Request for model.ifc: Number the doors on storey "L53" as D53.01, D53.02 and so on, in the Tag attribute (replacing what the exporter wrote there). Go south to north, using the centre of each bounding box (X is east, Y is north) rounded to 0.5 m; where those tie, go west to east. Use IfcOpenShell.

First a look at what the model holds.

```python
import ifcopenshell
import ifcopenshell.util.element
import ifcopenshell.util.placement

model = ifcopenshell.open("model.ifc")
print(model.schema)
storey = next(s for s in model.by_type("IfcBuildingStorey") if s.Name == "L53")
doors = [e for e in ifcopenshell.util.element.get_decomposition(storey) if e.is_a("IfcDoor")]
for e in sorted(doors, key=lambda e: e.id()):
    origin = ifcopenshell.util.placement.get_local_placement(e.ObjectPlacement)[:3, 3]
    print(e.id(), e.Tag, e.Name, origin.round(2) + 0.0, sep=" | ")
```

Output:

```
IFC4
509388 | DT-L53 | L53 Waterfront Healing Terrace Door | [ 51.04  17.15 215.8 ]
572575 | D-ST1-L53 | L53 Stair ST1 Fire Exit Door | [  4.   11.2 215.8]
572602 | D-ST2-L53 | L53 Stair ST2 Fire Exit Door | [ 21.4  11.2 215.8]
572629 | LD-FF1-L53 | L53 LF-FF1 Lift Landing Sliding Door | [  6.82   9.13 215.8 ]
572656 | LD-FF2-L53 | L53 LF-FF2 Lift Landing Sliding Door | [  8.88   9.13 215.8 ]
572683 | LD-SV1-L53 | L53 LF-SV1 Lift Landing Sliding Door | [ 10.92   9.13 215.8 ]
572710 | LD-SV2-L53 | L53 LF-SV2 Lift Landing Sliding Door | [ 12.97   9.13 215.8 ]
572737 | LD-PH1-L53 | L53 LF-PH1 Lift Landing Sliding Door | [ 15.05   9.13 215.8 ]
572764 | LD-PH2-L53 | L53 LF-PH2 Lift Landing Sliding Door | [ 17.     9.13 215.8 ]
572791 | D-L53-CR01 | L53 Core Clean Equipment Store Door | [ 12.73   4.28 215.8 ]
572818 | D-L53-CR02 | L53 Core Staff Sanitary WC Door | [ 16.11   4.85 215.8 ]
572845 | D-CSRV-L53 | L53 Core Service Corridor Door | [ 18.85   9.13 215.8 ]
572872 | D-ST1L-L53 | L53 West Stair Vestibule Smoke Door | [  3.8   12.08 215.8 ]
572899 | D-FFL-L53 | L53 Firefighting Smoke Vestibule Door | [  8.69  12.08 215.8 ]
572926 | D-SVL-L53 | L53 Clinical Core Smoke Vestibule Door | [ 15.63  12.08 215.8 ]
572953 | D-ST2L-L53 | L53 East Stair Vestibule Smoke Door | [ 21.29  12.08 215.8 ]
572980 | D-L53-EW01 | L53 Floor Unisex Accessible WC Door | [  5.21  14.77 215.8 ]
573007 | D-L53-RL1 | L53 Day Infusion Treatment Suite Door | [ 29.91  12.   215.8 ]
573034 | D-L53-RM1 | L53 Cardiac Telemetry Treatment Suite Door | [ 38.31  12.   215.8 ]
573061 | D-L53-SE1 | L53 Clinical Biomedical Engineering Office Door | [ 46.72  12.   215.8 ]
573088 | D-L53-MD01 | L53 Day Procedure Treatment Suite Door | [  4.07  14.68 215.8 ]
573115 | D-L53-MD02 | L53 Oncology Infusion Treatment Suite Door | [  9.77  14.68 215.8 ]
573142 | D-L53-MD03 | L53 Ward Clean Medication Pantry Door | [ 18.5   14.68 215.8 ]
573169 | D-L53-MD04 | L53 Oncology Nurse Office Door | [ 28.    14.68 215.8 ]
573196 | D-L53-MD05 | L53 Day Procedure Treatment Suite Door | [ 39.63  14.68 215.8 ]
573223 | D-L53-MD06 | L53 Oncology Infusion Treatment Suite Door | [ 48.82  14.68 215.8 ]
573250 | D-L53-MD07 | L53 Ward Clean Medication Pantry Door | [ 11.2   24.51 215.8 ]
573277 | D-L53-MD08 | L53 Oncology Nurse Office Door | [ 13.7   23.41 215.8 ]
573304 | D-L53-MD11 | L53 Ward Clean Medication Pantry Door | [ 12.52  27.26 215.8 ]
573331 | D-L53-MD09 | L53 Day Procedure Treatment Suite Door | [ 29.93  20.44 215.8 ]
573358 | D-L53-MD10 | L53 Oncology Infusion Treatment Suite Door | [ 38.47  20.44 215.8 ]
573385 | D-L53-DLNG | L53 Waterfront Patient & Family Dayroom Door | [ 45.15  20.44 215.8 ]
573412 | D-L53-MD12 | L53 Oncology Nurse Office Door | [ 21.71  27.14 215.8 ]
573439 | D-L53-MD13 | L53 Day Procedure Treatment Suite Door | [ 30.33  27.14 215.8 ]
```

```python
import ifcopenshell
import ifcopenshell.geom
import ifcopenshell.util.element
import ifcopenshell.util.shape

model = ifcopenshell.open("model.ifc")
settings = ifcopenshell.geom.settings()
settings.set("use-world-coords", True)


def centre(element):
    shape = ifcopenshell.geom.create_shape(settings, element)
    return ifcopenshell.util.shape.get_bbox_centroid(shape.geometry)


storey = next(s for s in model.by_type("IfcBuildingStorey") if s.Name == "L53")
doors = [e for e in ifcopenshell.util.element.get_decomposition(storey) if e.is_a("IfcDoor")]

# Insertion points can sit at a corner or the storey origin, so sort by the geometry (in metres).
centres = {e: centre(e) for e in doors}
doors.sort(key=lambda e: (round(centres[e][1] / 0.5), centres[e][0]))

for i, e in enumerate(doors, start=1):
    number = f"D53.{i:02d}"
    e.Tag = number
    print(e.id(), number)

model.write("model_edited.ifc")
```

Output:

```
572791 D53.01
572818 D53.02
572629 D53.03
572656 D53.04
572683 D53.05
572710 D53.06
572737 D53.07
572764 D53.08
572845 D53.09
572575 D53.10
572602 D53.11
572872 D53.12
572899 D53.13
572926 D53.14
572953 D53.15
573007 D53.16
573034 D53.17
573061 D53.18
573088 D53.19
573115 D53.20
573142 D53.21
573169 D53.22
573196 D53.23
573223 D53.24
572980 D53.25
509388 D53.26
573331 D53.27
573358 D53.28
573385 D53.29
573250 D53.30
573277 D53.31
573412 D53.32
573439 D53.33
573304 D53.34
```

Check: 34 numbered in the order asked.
